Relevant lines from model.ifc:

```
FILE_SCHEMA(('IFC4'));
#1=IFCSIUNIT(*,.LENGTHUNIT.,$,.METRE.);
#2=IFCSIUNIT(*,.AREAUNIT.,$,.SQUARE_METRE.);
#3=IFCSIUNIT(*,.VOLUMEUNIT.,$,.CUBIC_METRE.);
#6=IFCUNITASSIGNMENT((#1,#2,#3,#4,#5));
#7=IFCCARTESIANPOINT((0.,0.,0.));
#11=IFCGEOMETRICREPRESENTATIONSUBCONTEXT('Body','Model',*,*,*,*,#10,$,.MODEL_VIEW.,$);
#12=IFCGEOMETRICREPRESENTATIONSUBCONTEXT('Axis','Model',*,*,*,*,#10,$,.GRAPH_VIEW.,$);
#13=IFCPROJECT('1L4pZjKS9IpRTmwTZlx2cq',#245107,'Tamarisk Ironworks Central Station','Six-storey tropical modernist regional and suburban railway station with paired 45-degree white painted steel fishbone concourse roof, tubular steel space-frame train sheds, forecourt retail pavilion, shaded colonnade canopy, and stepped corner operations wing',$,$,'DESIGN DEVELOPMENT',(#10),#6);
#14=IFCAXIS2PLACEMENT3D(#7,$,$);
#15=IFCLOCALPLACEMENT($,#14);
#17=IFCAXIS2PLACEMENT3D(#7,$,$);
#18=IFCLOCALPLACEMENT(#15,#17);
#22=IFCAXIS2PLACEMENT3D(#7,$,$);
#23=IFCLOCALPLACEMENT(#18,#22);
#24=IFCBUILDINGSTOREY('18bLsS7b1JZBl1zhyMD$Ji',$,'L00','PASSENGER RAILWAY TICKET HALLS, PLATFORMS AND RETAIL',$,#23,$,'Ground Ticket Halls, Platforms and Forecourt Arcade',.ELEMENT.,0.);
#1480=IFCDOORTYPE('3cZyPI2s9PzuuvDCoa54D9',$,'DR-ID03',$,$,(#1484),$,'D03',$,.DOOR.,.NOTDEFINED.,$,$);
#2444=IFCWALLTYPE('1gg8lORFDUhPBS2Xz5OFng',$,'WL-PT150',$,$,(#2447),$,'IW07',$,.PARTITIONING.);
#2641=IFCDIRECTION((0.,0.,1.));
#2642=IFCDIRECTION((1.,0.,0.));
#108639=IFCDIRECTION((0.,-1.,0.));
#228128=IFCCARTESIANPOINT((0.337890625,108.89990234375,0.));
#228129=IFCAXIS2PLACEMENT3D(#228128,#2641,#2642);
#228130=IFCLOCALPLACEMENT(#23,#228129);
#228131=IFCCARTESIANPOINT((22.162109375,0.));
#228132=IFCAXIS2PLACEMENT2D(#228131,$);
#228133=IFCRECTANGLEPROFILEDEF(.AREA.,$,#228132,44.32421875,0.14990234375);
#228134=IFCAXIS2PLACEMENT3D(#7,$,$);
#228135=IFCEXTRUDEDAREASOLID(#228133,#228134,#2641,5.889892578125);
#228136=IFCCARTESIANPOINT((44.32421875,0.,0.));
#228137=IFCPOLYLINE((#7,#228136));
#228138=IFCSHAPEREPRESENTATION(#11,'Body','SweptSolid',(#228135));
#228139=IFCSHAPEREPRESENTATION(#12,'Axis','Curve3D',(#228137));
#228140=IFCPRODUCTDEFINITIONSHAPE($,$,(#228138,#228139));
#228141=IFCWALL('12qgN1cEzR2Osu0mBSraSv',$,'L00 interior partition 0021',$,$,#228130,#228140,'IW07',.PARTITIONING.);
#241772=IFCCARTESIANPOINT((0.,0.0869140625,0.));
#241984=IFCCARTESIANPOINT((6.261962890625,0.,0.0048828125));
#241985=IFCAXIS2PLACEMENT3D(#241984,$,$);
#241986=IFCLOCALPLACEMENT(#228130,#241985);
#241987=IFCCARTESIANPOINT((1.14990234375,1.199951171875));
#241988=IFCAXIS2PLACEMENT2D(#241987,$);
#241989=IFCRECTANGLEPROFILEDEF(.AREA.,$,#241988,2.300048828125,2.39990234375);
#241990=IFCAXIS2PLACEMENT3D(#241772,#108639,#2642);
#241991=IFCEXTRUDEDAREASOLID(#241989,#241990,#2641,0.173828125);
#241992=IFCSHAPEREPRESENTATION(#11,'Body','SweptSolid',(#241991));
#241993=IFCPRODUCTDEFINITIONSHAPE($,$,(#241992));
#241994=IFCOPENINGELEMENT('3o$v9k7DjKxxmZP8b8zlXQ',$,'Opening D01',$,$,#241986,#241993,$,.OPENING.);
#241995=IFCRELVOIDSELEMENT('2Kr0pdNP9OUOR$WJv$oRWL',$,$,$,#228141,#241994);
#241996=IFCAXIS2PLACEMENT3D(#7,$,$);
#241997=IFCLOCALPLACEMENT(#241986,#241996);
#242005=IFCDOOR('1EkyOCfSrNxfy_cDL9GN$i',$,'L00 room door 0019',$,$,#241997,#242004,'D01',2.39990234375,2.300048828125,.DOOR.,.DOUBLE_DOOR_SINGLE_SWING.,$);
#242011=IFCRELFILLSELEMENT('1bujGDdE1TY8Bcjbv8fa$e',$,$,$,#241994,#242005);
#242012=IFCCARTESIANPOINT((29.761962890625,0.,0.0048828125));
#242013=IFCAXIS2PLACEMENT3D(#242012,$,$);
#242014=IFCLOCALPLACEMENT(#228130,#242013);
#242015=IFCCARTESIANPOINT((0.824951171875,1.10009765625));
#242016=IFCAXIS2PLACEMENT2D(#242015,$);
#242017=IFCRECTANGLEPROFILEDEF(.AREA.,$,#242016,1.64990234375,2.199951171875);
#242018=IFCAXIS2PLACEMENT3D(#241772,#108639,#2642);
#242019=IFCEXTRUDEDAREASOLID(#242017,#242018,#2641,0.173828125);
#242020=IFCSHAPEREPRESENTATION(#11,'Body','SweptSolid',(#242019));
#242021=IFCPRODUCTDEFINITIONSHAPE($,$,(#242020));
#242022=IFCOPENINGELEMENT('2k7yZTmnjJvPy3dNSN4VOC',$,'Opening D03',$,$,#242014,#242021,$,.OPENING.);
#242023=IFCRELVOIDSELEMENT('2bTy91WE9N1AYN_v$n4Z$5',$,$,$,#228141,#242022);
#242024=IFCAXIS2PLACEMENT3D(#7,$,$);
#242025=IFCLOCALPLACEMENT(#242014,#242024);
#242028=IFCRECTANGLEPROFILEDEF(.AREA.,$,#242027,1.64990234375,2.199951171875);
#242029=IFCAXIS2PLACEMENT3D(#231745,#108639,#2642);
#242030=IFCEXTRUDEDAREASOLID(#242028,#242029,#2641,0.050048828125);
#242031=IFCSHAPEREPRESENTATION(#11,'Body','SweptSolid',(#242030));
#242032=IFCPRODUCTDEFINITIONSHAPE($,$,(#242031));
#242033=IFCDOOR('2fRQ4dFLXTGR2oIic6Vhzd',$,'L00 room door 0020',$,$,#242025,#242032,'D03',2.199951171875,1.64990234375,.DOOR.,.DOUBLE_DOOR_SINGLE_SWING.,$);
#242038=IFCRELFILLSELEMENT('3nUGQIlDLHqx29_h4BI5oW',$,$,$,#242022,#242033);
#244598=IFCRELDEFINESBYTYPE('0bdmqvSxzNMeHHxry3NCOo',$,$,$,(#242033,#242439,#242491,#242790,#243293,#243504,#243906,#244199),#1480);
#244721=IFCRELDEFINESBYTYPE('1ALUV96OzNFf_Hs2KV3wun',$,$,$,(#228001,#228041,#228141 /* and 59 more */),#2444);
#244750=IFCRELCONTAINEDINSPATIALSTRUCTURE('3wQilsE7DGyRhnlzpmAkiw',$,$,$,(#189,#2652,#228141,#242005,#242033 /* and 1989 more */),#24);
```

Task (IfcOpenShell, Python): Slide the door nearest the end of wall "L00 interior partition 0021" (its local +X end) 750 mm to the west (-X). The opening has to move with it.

```python
import ifcopenshell
import ifcopenshell.api.geometry
import ifcopenshell.util.placement
import ifcopenshell.util.unit

model = ifcopenshell.open("model.ifc")
unit_scale = ifcopenshell.util.unit.calculate_unit_scale(model)

door = model.by_id(242033)
opening = door.FillsVoids[0].RelatingOpeningElement
wall = opening.VoidsElements[0].RelatingBuildingElement

wall_matrix = ifcopenshell.util.placement.get_local_placement(wall.ObjectPlacement)
shift = wall_matrix[:3, 0] * -0.75 / unit_scale
before = ifcopenshell.util.placement.get_local_placement(door.ObjectPlacement)[:3, 3].copy()

# The door is placed relative to its opening, so it follows when the opening moves.
matrix = ifcopenshell.util.placement.get_local_placement(opening.ObjectPlacement)
matrix[:3, 3] += shift
ifcopenshell.api.geometry.edit_object_placement(
    model, product=opening, matrix=matrix, is_si=False, should_transform_children=True
)

after = ifcopenshell.util.placement.get_local_placement(door.ObjectPlacement)[:3, 3]
print("door moved by", (after - before).round(3) + 0.0)

model.write("model_updated.ifc")
```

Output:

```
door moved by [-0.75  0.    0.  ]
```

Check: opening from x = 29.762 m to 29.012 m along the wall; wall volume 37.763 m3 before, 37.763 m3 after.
